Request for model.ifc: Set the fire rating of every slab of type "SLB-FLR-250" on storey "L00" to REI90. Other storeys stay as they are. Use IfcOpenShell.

First a look at what the model holds.

```python
import ifcopenshell
import ifcopenshell.util.element

model = ifcopenshell.open("model.ifc")
print(model.schema)
storey = next(s for s in model.by_type("IfcBuildingStorey") if s.Name == "L00")
slabs = [e for e in ifcopenshell.util.element.get_decomposition(storey) if e.is_a("IfcSlab")]
seen = {}
for e in slabs:
    element_type = ifcopenshell.util.element.get_type(e)
    key = (element_type.Name if element_type != e and element_type else None, ifcopenshell.util.element.get_pset(e, "Pset_SlabCommon", "FireRating"))
    seen[key] = seen.get(key, 0) + 1
for (name, value), count in sorted(seen.items(), key=str):
    print(count, "x", name, "|", value)
```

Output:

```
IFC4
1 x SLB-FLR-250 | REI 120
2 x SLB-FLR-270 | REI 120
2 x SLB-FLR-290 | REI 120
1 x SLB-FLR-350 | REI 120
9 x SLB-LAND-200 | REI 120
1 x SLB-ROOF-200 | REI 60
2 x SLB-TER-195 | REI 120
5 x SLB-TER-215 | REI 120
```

```python
import ifcopenshell
import ifcopenshell.api.pset
import ifcopenshell.util.element

model = ifcopenshell.open("model.ifc")

storey = next(s for s in model.by_type("IfcBuildingStorey") if s.Name == "L00")
slabs = [e for e in ifcopenshell.util.element.get_decomposition(storey) if e.is_a("IfcSlab")]

count = 0
for e in slabs:
    element_type = ifcopenshell.util.element.get_type(e)
    if element_type in (None, e) or element_type.Name != "SLB-FLR-250":
        continue
    # add_pset returns the element's existing set when there is one.
    pset = ifcopenshell.api.pset.add_pset(model, product=e, name="Pset_SlabCommon")
    ifcopenshell.api.pset.edit_pset(model, pset=pset, properties={"FireRating": "REI90"})
    count += 1

print(count, "slabs updated")

model.write("model_updated.ifc")
```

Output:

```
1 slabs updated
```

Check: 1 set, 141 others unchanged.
